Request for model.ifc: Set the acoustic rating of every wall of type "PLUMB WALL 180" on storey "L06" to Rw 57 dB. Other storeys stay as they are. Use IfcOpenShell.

First a look at what the model holds.

```python
import ifcopenshell
import ifcopenshell.util.element

model = ifcopenshell.open("model.ifc")
print(model.schema)
storey = next(s for s in model.by_type("IfcBuildingStorey") if s.Name == "L06")
walls = [e for e in ifcopenshell.util.element.get_decomposition(storey) if e.is_a("IfcWall")]
seen = {}
for e in walls:
    element_type = ifcopenshell.util.element.get_type(e)
    key = (element_type.Name if element_type != e and element_type else None, ifcopenshell.util.element.get_pset(e, "Pset_WallCommon", "AcousticRating"))
    seen[key] = seen.get(key, 0) + 1
for (name, value), count in sorted(seen.items(), key=str):
    print(count, "x", name, "|", value)
```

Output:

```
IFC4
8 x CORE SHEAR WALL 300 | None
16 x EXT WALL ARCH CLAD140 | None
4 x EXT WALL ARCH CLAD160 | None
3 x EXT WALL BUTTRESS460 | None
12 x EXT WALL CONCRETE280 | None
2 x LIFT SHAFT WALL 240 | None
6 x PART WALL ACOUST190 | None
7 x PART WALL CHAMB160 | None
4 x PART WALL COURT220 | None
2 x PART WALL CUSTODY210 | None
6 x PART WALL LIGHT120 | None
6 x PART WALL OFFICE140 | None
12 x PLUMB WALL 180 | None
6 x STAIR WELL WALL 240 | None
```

```python
import ifcopenshell
import ifcopenshell.api.pset
import ifcopenshell.util.element

model = ifcopenshell.open("model.ifc")

storey = next(s for s in model.by_type("IfcBuildingStorey") if s.Name == "L06")
walls = [e for e in ifcopenshell.util.element.get_decomposition(storey) if e.is_a("IfcWall")]

count = 0
for e in walls:
    element_type = ifcopenshell.util.element.get_type(e)
    if element_type in (None, e) or element_type.Name != "PLUMB WALL 180":
        continue
    # add_pset returns the element's existing set when there is one.
    pset = ifcopenshell.api.pset.add_pset(model, product=e, name="Pset_WallCommon")
    ifcopenshell.api.pset.edit_pset(model, pset=pset, properties={"AcousticRating": "Rw 57 dB"})
    count += 1

print(count, "walls updated")

model.write("model_v2.ifc")
```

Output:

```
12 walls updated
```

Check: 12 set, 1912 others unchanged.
